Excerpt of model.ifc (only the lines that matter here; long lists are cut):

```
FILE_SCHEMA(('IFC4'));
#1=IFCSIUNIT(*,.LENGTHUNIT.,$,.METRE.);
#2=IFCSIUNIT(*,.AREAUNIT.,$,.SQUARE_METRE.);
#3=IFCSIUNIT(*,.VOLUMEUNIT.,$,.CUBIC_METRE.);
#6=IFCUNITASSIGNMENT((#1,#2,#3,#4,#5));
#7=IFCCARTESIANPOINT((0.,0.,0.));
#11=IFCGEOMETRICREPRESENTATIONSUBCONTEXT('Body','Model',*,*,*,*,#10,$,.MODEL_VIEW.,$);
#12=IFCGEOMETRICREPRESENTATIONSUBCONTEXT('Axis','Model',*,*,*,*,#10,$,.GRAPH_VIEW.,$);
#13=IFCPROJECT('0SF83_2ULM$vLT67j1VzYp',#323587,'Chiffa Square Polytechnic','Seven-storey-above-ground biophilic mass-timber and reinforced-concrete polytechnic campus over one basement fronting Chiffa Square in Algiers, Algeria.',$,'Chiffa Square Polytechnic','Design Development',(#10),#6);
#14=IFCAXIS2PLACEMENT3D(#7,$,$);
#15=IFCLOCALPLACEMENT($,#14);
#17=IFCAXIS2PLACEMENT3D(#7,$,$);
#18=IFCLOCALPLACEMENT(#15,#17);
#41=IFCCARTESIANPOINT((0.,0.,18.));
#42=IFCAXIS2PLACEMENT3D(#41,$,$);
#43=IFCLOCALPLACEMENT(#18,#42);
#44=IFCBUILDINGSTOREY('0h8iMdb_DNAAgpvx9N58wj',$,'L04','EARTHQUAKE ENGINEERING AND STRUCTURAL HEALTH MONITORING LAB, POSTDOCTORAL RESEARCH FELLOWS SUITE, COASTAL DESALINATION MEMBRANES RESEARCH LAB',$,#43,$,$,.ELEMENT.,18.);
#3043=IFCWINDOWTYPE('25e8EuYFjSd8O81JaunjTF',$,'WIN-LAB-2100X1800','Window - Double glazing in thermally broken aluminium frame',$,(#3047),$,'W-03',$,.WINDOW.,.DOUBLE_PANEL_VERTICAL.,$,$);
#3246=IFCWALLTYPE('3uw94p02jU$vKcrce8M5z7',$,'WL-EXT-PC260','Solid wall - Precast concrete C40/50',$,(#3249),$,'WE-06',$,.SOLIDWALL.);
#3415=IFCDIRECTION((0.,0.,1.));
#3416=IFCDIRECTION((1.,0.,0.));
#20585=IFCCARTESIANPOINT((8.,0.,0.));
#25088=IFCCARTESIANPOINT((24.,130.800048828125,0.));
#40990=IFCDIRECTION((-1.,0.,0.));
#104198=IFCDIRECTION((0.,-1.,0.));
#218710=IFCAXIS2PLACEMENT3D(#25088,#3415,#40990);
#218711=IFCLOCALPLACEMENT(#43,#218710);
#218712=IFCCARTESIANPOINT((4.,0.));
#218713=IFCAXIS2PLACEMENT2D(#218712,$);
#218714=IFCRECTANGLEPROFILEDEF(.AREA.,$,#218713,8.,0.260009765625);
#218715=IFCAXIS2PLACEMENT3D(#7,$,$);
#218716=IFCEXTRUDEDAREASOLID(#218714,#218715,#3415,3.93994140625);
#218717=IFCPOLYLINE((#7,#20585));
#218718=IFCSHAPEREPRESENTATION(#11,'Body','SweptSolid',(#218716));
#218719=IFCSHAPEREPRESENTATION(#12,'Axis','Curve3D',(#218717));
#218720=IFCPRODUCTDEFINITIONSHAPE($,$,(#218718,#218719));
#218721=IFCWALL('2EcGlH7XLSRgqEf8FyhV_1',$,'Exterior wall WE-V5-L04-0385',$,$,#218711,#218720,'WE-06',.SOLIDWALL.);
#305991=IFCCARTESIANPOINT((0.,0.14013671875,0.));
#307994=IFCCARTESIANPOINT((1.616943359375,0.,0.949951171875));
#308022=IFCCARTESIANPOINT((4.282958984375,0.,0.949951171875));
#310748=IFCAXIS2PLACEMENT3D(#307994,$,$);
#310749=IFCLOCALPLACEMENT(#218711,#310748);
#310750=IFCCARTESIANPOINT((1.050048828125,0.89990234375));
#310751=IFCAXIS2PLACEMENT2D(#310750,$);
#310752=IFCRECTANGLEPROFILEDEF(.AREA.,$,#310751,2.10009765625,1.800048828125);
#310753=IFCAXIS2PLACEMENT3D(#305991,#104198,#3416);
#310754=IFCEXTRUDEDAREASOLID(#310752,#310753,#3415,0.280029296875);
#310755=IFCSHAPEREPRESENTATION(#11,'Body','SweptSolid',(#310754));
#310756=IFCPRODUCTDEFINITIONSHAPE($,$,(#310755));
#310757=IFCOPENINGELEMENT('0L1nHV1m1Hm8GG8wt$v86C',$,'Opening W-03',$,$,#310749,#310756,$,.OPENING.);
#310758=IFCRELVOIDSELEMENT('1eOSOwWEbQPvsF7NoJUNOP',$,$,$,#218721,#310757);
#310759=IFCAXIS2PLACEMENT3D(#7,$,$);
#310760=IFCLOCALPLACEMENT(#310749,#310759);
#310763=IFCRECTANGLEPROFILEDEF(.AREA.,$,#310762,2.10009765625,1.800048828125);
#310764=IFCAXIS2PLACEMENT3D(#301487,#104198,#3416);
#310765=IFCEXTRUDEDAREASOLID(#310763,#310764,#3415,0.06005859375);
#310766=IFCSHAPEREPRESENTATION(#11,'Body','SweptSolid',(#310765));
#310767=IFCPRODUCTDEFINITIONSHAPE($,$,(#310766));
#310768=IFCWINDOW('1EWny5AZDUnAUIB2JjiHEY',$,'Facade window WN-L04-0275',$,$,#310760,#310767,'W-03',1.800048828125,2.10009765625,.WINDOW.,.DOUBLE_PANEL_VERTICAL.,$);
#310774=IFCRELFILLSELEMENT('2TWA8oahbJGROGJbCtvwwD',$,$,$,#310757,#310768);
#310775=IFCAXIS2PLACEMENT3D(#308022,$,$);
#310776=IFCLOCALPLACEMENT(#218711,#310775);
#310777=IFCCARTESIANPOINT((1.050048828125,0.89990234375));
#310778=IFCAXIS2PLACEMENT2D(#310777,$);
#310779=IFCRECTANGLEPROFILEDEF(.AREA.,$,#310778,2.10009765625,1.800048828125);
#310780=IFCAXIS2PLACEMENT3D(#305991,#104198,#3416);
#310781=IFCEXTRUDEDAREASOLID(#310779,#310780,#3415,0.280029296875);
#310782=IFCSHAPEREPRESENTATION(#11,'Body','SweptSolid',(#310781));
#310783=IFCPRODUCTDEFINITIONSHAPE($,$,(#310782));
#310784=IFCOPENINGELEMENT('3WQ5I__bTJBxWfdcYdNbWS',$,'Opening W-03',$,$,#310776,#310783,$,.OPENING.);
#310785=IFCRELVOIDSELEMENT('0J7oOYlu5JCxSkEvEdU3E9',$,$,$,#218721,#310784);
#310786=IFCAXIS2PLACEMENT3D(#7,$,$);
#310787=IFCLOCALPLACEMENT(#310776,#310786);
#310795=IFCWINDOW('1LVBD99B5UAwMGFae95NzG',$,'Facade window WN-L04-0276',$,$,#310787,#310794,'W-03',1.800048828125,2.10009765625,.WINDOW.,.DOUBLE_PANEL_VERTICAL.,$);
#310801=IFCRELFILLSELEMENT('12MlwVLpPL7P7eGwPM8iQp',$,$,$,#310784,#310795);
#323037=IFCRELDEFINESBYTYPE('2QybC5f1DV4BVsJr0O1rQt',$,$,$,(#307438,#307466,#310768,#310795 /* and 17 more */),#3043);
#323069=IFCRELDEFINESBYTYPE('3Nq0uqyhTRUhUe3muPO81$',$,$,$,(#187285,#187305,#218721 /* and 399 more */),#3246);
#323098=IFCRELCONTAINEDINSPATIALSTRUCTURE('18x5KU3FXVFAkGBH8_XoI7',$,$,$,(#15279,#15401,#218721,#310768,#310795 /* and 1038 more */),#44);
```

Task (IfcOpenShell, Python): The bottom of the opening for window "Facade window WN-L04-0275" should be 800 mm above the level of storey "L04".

```python
import numpy as np
import ifcopenshell
import ifcopenshell.api.geometry
import ifcopenshell.geom
import ifcopenshell.util.element
import ifcopenshell.util.placement
import ifcopenshell.util.shape
import ifcopenshell.util.unit

model = ifcopenshell.open("model.ifc")
unit_scale = ifcopenshell.util.unit.calculate_unit_scale(model)

window = model.by_guid("1EWny5AZDUnAUIB2JjiHEY")
opening = window.FillsVoids[0].RelatingOpeningElement
storey = ifcopenshell.util.element.get_container(window, ifc_class="IfcBuildingStorey")
level = ifcopenshell.util.placement.get_local_placement(storey.ObjectPlacement)[2, 3]

# The opening's origin need not be at the sill, so measure its lowest point.
shape = ifcopenshell.geom.create_shape(ifcopenshell.geom.settings(), opening)
bottom = ifcopenshell.util.shape.get_shape_bottom_elevation(shape, shape.geometry) / unit_scale
dz = level + 0.8 / unit_scale - bottom

shift = np.array([0.0, 0.0, dz])
# The window is placed relative to its opening, so it follows when the opening moves.
matrix = ifcopenshell.util.placement.get_local_placement(opening.ObjectPlacement)
matrix[:3, 3] += shift
ifcopenshell.api.geometry.edit_object_placement(
    model, product=opening, matrix=matrix, is_si=False, should_transform_children=True
)

print(f"moved by {dz * unit_scale:+.3f} m")

model.write("model-out.ifc")
```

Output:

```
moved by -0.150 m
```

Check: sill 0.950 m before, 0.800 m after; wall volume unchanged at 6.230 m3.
